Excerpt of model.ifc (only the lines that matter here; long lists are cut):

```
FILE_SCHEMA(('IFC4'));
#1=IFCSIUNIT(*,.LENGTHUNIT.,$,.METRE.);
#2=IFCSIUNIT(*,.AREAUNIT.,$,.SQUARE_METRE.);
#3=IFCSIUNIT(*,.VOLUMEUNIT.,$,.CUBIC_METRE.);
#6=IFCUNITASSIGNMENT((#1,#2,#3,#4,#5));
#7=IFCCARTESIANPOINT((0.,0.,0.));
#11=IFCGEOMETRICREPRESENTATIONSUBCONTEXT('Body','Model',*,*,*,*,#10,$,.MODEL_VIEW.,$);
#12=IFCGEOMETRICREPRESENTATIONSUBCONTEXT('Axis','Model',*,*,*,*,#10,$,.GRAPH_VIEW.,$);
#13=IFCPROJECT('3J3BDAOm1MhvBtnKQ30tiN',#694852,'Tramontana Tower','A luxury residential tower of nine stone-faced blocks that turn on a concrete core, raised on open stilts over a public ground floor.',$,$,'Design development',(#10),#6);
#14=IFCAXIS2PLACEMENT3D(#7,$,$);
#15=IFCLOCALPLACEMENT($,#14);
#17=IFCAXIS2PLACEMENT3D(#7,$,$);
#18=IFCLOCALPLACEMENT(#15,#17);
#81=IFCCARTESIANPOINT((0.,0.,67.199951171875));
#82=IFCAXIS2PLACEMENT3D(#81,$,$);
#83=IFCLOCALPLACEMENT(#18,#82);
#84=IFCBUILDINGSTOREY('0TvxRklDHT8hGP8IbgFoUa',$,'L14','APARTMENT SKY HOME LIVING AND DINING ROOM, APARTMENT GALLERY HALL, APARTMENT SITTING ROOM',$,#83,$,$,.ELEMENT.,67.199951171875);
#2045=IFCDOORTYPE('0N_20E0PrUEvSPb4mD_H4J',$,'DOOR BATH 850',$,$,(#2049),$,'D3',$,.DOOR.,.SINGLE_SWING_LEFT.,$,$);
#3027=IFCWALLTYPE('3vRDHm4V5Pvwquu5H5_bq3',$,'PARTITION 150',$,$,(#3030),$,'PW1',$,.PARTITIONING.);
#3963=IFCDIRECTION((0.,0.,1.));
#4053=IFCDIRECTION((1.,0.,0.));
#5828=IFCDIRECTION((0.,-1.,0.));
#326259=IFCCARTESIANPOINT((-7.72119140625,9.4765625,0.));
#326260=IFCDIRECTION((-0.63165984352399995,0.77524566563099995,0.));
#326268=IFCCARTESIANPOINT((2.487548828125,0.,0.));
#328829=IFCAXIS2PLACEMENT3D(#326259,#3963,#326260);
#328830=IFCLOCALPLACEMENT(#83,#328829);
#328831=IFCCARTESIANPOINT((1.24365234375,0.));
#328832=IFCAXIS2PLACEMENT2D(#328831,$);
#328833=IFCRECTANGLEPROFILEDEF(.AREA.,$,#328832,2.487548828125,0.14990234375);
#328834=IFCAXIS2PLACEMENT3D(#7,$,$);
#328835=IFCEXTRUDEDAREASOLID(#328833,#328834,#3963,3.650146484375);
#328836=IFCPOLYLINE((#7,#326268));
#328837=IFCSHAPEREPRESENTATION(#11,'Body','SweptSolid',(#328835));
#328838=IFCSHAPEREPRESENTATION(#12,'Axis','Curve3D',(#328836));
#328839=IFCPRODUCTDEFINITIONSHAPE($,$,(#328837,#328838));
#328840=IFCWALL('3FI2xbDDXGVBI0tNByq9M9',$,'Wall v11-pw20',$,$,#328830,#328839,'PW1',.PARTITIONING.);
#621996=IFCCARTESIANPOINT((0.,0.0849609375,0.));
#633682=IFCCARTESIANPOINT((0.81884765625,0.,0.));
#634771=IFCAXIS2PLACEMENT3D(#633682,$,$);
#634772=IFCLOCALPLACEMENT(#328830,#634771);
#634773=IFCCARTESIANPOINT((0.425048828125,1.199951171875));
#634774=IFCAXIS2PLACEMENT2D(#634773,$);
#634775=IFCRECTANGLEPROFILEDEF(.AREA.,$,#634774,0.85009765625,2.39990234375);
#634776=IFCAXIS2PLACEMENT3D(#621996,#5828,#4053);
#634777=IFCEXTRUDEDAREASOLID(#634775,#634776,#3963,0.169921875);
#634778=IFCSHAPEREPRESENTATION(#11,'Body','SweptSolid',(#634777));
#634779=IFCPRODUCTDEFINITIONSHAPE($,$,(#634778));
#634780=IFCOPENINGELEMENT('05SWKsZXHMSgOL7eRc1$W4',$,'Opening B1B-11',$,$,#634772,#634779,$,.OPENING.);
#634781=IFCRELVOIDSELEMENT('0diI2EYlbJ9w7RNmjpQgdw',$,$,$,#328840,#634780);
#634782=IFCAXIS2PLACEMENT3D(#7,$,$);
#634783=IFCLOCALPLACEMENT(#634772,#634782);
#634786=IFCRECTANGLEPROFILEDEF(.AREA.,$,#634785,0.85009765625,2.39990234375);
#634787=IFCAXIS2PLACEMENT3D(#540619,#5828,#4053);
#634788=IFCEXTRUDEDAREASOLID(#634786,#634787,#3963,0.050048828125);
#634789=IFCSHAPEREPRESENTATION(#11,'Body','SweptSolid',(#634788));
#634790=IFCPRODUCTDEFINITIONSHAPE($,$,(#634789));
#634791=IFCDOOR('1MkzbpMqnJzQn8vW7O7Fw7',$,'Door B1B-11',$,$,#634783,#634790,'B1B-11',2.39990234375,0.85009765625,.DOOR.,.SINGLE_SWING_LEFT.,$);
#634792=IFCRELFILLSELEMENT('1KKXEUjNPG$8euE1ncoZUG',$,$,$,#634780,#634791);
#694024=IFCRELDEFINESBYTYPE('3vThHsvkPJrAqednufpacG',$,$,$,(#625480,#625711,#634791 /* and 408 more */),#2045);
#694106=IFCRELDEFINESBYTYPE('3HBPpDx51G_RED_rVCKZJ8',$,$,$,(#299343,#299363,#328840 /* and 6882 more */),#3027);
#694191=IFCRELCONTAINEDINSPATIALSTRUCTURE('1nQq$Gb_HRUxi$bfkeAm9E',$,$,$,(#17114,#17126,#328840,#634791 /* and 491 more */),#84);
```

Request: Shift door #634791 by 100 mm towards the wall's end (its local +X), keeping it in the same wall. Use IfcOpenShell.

```python
import ifcopenshell
import ifcopenshell.api.geometry
import ifcopenshell.util.placement

model = ifcopenshell.open("model.ifc")

door = model.by_guid("1MkzbpMqnJzQn8vW7O7Fw7")
opening = door.FillsVoids[0].RelatingOpeningElement
wall = opening.VoidsElements[0].RelatingBuildingElement

wall_matrix = ifcopenshell.util.placement.get_local_placement(wall.ObjectPlacement)
shift = wall_matrix[:3, 0] * 0.1
before = ifcopenshell.util.placement.get_local_placement(door.ObjectPlacement)[:3, 3].copy()

# The door is placed relative to its opening, so it follows when the opening moves.
matrix = ifcopenshell.util.placement.get_local_placement(opening.ObjectPlacement)
matrix[:3, 3] += shift
ifcopenshell.api.geometry.edit_object_placement(
    model, product=opening, matrix=matrix, is_si=False, should_transform_children=True
)

after = ifcopenshell.util.placement.get_local_placement(door.ObjectPlacement)[:3, 3]
print("door moved by", (after - before).round(3) + 0.0)

model.write("model_updated.ifc")
```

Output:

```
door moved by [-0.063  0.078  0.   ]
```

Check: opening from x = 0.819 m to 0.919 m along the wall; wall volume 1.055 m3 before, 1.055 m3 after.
